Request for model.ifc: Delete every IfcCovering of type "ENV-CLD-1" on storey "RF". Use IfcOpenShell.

First a look at what the model holds.

```python
import ifcopenshell
import ifcopenshell.util.element

model = ifcopenshell.open("model.ifc")
print(model.schema)
storey = next(s for s in model.by_type("IfcBuildingStorey") if s.Name == "RF")
coverings = [e for e in ifcopenshell.util.element.get_decomposition(storey) if e.is_a("IfcCovering")]
seen = {}
for e in coverings:
    element_type = ifcopenshell.util.element.get_type(e)
    name = element_type.Name if element_type not in (None, e) else None
    seen[name] = seen.get(name, 0) + 1
for name, count in sorted(seen.items(), key=str):
    print(count, "x", name)
```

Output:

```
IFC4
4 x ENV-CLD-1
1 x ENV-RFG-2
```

```python
import ifcopenshell
import ifcopenshell.api.root
import ifcopenshell.util.element

model = ifcopenshell.open("model.ifc")

storey = next(s for s in model.by_type("IfcBuildingStorey") if s.Name == "RF")
coverings = [e for e in ifcopenshell.util.element.get_decomposition(storey) if e.is_a("IfcCovering")]
targets = [e for e in coverings if (t := ifcopenshell.util.element.get_type(e)) not in (None, e) and t.Name == "ENV-CLD-1"]

for e in targets:
    ifcopenshell.api.root.remove_product(model, product=e)
print(len(targets), "removed")

model.write("model_updated.ifc")
```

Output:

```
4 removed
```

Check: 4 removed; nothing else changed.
